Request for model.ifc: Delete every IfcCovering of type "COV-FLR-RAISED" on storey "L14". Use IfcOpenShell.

First a look at what the model holds.

```python
import ifcopenshell
import ifcopenshell.util.element

model = ifcopenshell.open("model.ifc")
print(model.schema)
storey = next(s for s in model.by_type("IfcBuildingStorey") if s.Name == "L14")
coverings = [e for e in ifcopenshell.util.element.get_decomposition(storey) if e.is_a("IfcCovering")]
seen = {}
for e in coverings:
    element_type = ifcopenshell.util.element.get_type(e)
    name = element_type.Name if element_type not in (None, e) else None
    seen[name] = seen.get(name, 0) + 1
for name, count in sorted(seen.items(), key=str):
    print(count, "x", name)
```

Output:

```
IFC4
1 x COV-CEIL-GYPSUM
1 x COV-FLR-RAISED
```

```python
import ifcopenshell
import ifcopenshell.api.root
import ifcopenshell.util.element

model = ifcopenshell.open("model.ifc")

storey = next(s for s in model.by_type("IfcBuildingStorey") if s.Name == "L14")
coverings = [e for e in ifcopenshell.util.element.get_decomposition(storey) if e.is_a("IfcCovering")]
targets = [e for e in coverings if (t := ifcopenshell.util.element.get_type(e)) not in (None, e) and t.Name == "COV-FLR-RAISED"]

for e in targets:
    ifcopenshell.api.root.remove_product(model, product=e)
print(len(targets), "removed")

model.write("model-out.ifc")
```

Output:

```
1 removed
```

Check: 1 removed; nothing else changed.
